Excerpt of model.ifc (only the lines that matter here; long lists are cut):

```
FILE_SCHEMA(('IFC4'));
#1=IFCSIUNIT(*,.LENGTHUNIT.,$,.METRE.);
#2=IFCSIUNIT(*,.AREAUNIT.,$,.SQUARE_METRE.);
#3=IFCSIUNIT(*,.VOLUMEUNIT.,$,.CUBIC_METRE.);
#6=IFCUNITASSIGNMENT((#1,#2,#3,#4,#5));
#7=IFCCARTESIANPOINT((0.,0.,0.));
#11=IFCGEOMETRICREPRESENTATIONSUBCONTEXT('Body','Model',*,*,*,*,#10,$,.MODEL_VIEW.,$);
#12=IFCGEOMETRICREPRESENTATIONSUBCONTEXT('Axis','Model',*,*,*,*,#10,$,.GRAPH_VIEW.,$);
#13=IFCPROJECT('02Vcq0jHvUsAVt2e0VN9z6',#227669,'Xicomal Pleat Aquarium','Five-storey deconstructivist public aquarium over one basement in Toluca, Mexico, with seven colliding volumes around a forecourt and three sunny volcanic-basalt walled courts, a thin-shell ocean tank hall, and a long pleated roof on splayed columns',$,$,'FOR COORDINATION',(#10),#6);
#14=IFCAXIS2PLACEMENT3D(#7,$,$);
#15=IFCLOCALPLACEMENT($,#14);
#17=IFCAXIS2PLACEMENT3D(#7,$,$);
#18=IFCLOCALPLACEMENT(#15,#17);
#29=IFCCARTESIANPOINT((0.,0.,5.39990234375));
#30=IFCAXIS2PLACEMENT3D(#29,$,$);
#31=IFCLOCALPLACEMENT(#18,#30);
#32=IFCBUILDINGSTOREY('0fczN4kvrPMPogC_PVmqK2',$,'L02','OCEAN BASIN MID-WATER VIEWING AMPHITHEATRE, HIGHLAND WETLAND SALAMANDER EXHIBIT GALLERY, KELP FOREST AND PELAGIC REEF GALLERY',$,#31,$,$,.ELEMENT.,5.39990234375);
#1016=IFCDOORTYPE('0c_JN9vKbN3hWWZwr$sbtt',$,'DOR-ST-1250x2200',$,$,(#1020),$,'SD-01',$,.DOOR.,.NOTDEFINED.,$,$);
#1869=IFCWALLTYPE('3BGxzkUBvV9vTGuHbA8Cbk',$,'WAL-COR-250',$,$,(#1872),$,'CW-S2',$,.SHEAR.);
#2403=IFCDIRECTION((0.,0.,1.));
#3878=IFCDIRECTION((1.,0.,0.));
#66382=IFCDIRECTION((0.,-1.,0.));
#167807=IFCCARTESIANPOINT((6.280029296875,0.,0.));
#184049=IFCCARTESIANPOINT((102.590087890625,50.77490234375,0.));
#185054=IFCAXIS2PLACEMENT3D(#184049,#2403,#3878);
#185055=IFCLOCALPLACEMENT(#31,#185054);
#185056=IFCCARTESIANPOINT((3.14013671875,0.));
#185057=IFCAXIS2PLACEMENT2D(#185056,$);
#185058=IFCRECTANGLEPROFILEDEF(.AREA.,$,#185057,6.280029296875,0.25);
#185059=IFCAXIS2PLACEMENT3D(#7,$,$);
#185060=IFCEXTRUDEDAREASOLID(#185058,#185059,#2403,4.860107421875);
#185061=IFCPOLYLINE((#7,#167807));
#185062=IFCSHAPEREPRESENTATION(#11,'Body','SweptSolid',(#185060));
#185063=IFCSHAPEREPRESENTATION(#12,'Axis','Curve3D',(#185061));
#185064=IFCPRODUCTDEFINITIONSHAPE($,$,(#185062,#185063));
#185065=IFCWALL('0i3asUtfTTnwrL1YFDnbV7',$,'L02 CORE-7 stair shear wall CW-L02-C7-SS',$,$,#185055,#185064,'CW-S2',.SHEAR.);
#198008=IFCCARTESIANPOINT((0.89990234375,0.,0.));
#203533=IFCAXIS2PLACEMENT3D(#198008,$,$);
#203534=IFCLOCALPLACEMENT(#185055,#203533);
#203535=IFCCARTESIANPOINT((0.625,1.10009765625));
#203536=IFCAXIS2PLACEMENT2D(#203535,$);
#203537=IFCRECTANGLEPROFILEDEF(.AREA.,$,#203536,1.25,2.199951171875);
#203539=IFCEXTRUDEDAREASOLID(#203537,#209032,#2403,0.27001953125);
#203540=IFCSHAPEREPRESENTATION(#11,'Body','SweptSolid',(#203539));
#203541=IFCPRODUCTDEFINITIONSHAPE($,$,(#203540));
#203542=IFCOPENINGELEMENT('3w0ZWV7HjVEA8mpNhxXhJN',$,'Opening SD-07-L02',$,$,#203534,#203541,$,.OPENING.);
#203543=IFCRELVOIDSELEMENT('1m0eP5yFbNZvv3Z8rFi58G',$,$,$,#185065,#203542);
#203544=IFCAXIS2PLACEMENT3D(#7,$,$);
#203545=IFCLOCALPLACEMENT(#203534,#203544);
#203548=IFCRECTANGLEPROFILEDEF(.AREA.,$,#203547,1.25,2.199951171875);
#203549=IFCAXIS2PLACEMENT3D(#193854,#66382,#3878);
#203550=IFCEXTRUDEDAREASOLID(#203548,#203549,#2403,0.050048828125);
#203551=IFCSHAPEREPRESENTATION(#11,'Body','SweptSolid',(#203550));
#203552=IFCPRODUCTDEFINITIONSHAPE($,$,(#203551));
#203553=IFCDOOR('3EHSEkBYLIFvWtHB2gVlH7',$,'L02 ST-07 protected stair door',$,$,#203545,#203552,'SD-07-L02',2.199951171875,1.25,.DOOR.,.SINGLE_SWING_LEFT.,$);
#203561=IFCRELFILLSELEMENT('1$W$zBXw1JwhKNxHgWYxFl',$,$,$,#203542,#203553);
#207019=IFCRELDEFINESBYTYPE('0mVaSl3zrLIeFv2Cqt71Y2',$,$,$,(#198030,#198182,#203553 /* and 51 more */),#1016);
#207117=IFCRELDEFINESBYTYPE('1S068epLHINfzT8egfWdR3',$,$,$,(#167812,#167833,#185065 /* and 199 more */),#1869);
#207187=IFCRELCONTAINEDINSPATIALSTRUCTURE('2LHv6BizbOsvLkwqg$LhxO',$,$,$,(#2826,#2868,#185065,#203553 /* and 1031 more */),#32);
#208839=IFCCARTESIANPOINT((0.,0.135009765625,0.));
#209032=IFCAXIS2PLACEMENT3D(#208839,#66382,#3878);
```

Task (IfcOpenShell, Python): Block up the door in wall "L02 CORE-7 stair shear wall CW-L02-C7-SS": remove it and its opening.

```python
import ifcopenshell
import ifcopenshell.api.feature
import ifcopenshell.api.root
import ifcopenshell.geom
import ifcopenshell.util.shape

model = ifcopenshell.open("model.ifc")
settings = ifcopenshell.geom.settings()


def volume(element):
    """Net volume in cubic metres, openings subtracted."""
    shape = ifcopenshell.geom.create_shape(settings, element)
    return ifcopenshell.util.shape.get_volume(shape.geometry)


door = model.by_guid("3EHSEkBYLIFvWtHB2gVlH7")
opening = door.FillsVoids[0].RelatingOpeningElement
wall = opening.VoidsElements[0].RelatingBuildingElement
before = volume(wall)

ifcopenshell.api.root.remove_product(model, product=door)
ifcopenshell.api.feature.remove_feature(model, feature=opening)

after = volume(wall)

print(f"wall volume {before:.3f} -> {after:.3f} m3")

model.write("model_v2.ifc")
```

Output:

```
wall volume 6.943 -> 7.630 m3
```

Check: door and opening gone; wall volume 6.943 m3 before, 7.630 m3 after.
